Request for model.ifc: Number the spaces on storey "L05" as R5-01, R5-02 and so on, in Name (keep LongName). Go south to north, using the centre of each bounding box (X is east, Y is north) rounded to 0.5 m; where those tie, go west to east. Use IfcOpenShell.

First a look at what the model holds.

```python
import ifcopenshell
import ifcopenshell.util.element
import ifcopenshell.util.placement

model = ifcopenshell.open("model.ifc")
print(model.schema)
storey = next(s for s in model.by_type("IfcBuildingStorey") if s.Name == "L05")
spaces = [e for e in ifcopenshell.util.element.get_decomposition(storey) if e.is_a("IfcSpace")]
for e in sorted(spaces, key=lambda e: e.id()):
    origin = ifcopenshell.util.placement.get_local_placement(e.ObjectPlacement)[:3, 3]
    print(e.id(), e.Name, e.LongName, origin.round(2) + 0.0, sep=" | ")
```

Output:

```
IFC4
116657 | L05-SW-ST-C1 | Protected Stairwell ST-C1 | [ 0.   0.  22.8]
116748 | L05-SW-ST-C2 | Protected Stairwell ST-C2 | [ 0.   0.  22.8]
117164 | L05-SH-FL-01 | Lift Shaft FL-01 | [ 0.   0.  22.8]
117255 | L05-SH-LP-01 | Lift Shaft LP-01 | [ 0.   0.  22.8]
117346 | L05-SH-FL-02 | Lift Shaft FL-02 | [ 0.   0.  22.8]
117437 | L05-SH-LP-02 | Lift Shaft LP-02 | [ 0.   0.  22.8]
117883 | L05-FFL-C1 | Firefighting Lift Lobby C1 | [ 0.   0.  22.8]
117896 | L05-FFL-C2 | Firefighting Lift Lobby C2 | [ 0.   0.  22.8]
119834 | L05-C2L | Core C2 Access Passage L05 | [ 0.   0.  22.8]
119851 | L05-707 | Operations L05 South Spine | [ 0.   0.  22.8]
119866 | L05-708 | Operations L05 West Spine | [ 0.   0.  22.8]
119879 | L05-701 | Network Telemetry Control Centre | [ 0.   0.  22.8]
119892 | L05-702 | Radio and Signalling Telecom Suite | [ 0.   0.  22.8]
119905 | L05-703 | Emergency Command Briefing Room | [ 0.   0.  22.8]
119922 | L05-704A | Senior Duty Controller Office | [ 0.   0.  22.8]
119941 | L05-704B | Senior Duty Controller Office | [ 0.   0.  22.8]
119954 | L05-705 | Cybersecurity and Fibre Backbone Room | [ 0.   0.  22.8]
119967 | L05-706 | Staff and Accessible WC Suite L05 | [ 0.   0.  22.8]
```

```python
import ifcopenshell
import ifcopenshell.geom
import ifcopenshell.util.element
import ifcopenshell.util.shape

model = ifcopenshell.open("model.ifc")
settings = ifcopenshell.geom.settings()
settings.set("use-world-coords", True)


def centre(element):
    shape = ifcopenshell.geom.create_shape(settings, element)
    return ifcopenshell.util.shape.get_bbox_centroid(shape.geometry)


storey = next(s for s in model.by_type("IfcBuildingStorey") if s.Name == "L05")
spaces = [e for e in ifcopenshell.util.element.get_decomposition(storey) if e.is_a("IfcSpace")]

# Insertion points can sit at a corner or the storey origin, so sort by the geometry (in metres).
centres = {e: centre(e) for e in spaces}
spaces.sort(key=lambda e: (round(centres[e][1] / 0.5), centres[e][0]))

for i, e in enumerate(spaces, start=1):
    number = f"R5-{i:02d}"
    e.Name = number
    print(e.id(), number)

model.write("model_edited.ifc")
```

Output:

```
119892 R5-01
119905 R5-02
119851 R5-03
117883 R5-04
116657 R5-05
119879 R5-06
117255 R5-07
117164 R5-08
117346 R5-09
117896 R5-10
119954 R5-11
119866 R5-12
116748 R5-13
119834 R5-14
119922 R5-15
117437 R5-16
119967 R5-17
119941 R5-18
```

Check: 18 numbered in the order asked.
